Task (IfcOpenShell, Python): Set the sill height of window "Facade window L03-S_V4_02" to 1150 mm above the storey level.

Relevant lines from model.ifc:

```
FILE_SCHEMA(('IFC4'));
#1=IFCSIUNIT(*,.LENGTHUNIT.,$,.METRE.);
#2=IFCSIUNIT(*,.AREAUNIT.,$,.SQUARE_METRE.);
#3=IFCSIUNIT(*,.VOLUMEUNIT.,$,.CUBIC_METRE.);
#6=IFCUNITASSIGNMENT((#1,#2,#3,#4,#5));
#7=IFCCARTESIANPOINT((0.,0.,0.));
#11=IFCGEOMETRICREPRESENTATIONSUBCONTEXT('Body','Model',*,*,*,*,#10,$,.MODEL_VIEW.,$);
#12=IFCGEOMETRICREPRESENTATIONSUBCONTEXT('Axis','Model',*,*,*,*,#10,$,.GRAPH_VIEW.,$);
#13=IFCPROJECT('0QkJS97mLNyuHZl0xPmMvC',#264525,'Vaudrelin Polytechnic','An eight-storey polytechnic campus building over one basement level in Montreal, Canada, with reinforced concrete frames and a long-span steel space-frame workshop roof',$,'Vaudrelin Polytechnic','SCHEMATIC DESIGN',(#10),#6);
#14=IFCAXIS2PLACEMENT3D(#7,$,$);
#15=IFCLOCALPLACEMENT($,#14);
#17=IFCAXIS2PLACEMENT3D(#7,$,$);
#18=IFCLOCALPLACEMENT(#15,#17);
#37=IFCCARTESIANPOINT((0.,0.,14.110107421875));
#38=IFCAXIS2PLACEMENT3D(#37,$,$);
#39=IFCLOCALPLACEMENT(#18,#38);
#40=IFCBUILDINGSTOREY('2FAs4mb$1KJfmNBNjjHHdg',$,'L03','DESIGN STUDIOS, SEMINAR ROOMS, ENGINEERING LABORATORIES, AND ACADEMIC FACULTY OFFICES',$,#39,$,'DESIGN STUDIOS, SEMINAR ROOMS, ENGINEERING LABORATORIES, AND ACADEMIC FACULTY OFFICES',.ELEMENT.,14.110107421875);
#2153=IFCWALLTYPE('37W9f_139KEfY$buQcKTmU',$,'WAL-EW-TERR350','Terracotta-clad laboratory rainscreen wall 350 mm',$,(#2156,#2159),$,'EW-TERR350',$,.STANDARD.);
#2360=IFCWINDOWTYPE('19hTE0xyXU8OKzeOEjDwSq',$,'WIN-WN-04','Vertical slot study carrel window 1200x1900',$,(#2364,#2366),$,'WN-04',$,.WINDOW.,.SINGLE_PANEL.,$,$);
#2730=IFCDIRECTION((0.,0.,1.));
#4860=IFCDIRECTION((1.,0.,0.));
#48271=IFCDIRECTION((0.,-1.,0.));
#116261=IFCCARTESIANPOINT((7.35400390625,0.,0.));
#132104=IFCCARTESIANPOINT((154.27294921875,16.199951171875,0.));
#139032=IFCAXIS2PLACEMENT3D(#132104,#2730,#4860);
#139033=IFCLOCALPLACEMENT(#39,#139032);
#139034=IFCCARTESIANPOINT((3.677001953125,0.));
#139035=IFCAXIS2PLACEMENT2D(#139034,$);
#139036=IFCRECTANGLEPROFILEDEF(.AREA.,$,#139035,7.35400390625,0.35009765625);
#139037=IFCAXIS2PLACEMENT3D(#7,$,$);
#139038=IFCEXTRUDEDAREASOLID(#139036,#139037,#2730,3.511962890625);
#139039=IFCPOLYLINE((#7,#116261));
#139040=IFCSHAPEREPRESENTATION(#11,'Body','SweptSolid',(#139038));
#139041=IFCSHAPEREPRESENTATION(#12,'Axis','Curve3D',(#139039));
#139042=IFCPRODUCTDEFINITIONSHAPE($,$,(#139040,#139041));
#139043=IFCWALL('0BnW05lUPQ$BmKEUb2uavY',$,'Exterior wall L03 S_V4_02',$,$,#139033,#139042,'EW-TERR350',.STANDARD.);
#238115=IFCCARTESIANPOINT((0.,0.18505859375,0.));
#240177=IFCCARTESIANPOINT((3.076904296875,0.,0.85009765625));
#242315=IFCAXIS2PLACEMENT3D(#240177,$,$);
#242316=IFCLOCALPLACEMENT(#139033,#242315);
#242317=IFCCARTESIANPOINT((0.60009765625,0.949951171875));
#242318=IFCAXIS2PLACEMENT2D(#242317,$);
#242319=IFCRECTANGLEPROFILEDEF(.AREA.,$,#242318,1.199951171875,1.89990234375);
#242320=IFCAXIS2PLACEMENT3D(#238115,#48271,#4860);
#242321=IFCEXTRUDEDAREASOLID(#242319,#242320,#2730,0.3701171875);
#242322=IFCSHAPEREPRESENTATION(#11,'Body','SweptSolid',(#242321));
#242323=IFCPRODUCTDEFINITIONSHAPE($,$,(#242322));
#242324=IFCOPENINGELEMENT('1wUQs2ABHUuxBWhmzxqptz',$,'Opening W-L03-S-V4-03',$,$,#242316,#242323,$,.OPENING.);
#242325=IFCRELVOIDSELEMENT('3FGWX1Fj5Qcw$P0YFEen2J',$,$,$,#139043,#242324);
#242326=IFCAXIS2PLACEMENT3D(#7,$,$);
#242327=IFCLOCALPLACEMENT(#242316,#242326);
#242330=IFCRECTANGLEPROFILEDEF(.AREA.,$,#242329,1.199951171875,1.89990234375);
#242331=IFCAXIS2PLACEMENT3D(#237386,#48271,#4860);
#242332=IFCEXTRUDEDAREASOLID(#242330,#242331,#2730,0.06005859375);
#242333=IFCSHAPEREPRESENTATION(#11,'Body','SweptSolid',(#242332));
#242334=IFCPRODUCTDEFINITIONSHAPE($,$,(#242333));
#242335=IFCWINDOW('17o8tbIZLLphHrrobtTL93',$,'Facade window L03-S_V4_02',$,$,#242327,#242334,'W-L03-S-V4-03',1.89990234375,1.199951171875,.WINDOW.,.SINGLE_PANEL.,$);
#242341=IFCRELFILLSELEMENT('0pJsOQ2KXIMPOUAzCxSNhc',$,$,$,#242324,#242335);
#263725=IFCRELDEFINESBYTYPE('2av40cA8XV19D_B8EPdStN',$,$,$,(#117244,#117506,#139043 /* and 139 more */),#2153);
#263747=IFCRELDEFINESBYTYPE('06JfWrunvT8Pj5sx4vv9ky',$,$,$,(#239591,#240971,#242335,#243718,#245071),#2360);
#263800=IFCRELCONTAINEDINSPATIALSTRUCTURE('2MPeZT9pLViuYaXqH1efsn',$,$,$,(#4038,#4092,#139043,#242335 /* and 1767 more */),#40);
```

```python
import numpy as np
import ifcopenshell
import ifcopenshell.api.geometry
import ifcopenshell.geom
import ifcopenshell.util.element
import ifcopenshell.util.placement
import ifcopenshell.util.shape
import ifcopenshell.util.unit

model = ifcopenshell.open("model.ifc")
unit_scale = ifcopenshell.util.unit.calculate_unit_scale(model)

window = model.by_guid("17o8tbIZLLphHrrobtTL93")
opening = window.FillsVoids[0].RelatingOpeningElement
storey = ifcopenshell.util.element.get_container(window, ifc_class="IfcBuildingStorey")
level = ifcopenshell.util.placement.get_local_placement(storey.ObjectPlacement)[2, 3]

# The opening's origin need not be at the sill, so measure its lowest point.
shape = ifcopenshell.geom.create_shape(ifcopenshell.geom.settings(), opening)
bottom = ifcopenshell.util.shape.get_shape_bottom_elevation(shape, shape.geometry) / unit_scale
dz = level + 1.15 / unit_scale - bottom

shift = np.array([0.0, 0.0, dz])
# The window is placed relative to its opening, so it follows when the opening moves.
matrix = ifcopenshell.util.placement.get_local_placement(opening.ObjectPlacement)
matrix[:3, 3] += shift
ifcopenshell.api.geometry.edit_object_placement(
    model, product=opening, matrix=matrix, is_si=False, should_transform_children=True
)

print(f"moved by {dz * unit_scale:+.3f} m")

model.write("model_updated.ifc")
```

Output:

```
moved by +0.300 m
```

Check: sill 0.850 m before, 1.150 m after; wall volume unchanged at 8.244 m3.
